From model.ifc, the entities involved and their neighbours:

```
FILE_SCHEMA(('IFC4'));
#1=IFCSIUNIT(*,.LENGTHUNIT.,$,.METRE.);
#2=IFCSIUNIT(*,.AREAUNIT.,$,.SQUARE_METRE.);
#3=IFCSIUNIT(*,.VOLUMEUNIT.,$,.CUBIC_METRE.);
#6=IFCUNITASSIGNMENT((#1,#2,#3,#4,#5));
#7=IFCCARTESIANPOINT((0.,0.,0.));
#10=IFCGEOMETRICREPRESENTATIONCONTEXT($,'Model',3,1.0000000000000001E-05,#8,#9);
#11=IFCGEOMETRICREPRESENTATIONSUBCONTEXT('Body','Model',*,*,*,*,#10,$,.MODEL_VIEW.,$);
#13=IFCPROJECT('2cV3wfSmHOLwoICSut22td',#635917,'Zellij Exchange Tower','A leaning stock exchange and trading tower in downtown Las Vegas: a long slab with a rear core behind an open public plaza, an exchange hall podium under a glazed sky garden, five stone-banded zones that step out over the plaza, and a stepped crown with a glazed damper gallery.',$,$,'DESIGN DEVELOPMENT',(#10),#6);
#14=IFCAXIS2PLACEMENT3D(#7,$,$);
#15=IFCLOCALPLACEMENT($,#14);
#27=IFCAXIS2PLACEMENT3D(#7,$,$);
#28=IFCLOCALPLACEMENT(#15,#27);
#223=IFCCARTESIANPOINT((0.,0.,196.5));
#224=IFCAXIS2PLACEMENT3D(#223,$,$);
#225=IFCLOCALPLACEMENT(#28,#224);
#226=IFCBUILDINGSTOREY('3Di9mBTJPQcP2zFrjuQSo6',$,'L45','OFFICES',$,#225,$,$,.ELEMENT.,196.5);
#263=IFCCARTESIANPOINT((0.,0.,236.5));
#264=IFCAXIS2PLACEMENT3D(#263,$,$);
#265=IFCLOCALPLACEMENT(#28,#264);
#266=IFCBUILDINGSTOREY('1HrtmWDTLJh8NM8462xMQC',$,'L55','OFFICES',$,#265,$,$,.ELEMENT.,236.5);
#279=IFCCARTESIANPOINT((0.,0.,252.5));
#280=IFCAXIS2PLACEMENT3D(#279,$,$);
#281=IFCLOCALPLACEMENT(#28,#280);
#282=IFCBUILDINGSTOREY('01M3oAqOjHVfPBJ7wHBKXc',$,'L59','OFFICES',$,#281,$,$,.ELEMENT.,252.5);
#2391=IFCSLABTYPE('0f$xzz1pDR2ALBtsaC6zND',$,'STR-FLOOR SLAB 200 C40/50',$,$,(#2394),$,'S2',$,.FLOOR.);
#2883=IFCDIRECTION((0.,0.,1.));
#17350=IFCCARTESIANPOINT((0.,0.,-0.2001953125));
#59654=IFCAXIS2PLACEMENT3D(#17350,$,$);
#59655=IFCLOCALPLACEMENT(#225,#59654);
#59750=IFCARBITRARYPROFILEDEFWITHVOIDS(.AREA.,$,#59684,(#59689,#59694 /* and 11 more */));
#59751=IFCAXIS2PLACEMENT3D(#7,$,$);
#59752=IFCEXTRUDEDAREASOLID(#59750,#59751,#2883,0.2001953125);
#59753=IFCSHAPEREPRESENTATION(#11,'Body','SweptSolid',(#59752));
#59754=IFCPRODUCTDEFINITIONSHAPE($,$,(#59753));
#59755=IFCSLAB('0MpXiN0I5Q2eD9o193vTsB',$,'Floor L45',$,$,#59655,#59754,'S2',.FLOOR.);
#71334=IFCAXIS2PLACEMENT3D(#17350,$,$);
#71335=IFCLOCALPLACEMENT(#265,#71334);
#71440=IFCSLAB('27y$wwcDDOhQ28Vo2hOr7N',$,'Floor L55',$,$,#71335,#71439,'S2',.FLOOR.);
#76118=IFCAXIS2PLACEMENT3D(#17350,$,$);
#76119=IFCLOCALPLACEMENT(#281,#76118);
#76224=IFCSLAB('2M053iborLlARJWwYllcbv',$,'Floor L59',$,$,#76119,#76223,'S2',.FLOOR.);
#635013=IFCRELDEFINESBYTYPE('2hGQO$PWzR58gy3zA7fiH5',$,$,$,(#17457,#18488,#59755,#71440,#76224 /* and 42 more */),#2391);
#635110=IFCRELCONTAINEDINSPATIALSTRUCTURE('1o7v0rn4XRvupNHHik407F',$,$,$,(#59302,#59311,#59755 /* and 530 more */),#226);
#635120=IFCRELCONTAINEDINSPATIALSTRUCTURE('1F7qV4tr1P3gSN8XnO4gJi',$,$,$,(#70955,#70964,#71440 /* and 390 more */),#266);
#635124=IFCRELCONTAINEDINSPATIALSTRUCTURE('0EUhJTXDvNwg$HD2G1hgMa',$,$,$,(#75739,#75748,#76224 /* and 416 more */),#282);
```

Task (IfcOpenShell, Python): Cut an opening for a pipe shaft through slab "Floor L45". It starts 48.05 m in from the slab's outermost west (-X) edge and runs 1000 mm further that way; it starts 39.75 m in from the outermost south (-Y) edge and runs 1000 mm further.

```python
import numpy as np
import ifcopenshell
import ifcopenshell.api.feature
import ifcopenshell.api.geometry
import ifcopenshell.api.root
import ifcopenshell.geom
import ifcopenshell.util.placement
import ifcopenshell.util.representation
import ifcopenshell.util.shape
import ifcopenshell.util.unit

model = ifcopenshell.open("model.ifc")
unit_scale = ifcopenshell.util.unit.calculate_unit_scale(model)
settings = ifcopenshell.geom.settings()


def volume(element):
    """Net volume in cubic metres, openings subtracted."""
    shape = ifcopenshell.geom.create_shape(settings, element)
    return ifcopenshell.util.shape.get_volume(shape.geometry)


slab = model.by_guid("0MpXiN0I5Q2eD9o193vTsB")
before = volume(slab)

# Extent in the slab's own axes, in metres. The edges named are its -X and -Y sides.
slab_shape = ifcopenshell.geom.create_shape(settings, slab)
vertices = ifcopenshell.util.shape.get_vertices(slab_shape.geometry)
x_min, y_min, bottom = vertices.min(axis=0)
top = vertices[:, 2].max()

opening = ifcopenshell.api.root.create_entity(model, ifc_class="IfcOpeningElement", name="Pipe shaft opening", predefined_type="OPENING")
context = ifcopenshell.util.representation.get_context(model, "Model", "Body", "MODEL_VIEW")
width, depth = 1, 1
outline = [(0.0, 0.0), (width, 0.0), (width, depth), (0.0, depth), (0.0, 0.0)]
# Overshoot both faces by 50 mm so the cut is clean.
shape = ifcopenshell.api.geometry.add_slab_representation(
    model, context=context, depth=top - bottom + 0.1, polyline=outline
)
ifcopenshell.api.geometry.assign_representation(model, product=opening, representation=shape)

matrix = ifcopenshell.util.placement.get_local_placement(slab.ObjectPlacement)
matrix[:, 3] = matrix @ np.append(np.array([x_min + 48.05, y_min + 39.75, bottom - 0.05]) / unit_scale, 1.0)
ifcopenshell.api.geometry.edit_object_placement(model, product=opening, matrix=matrix, is_si=False)
ifcopenshell.api.feature.add_feature(model, feature=opening, element=slab)

after = volume(slab)

print(f"slab volume {before:.3f} -> {after:.3f} m3")

model.write("model_updated.ifc")
```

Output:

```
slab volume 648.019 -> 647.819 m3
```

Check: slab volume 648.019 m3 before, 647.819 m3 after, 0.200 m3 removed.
